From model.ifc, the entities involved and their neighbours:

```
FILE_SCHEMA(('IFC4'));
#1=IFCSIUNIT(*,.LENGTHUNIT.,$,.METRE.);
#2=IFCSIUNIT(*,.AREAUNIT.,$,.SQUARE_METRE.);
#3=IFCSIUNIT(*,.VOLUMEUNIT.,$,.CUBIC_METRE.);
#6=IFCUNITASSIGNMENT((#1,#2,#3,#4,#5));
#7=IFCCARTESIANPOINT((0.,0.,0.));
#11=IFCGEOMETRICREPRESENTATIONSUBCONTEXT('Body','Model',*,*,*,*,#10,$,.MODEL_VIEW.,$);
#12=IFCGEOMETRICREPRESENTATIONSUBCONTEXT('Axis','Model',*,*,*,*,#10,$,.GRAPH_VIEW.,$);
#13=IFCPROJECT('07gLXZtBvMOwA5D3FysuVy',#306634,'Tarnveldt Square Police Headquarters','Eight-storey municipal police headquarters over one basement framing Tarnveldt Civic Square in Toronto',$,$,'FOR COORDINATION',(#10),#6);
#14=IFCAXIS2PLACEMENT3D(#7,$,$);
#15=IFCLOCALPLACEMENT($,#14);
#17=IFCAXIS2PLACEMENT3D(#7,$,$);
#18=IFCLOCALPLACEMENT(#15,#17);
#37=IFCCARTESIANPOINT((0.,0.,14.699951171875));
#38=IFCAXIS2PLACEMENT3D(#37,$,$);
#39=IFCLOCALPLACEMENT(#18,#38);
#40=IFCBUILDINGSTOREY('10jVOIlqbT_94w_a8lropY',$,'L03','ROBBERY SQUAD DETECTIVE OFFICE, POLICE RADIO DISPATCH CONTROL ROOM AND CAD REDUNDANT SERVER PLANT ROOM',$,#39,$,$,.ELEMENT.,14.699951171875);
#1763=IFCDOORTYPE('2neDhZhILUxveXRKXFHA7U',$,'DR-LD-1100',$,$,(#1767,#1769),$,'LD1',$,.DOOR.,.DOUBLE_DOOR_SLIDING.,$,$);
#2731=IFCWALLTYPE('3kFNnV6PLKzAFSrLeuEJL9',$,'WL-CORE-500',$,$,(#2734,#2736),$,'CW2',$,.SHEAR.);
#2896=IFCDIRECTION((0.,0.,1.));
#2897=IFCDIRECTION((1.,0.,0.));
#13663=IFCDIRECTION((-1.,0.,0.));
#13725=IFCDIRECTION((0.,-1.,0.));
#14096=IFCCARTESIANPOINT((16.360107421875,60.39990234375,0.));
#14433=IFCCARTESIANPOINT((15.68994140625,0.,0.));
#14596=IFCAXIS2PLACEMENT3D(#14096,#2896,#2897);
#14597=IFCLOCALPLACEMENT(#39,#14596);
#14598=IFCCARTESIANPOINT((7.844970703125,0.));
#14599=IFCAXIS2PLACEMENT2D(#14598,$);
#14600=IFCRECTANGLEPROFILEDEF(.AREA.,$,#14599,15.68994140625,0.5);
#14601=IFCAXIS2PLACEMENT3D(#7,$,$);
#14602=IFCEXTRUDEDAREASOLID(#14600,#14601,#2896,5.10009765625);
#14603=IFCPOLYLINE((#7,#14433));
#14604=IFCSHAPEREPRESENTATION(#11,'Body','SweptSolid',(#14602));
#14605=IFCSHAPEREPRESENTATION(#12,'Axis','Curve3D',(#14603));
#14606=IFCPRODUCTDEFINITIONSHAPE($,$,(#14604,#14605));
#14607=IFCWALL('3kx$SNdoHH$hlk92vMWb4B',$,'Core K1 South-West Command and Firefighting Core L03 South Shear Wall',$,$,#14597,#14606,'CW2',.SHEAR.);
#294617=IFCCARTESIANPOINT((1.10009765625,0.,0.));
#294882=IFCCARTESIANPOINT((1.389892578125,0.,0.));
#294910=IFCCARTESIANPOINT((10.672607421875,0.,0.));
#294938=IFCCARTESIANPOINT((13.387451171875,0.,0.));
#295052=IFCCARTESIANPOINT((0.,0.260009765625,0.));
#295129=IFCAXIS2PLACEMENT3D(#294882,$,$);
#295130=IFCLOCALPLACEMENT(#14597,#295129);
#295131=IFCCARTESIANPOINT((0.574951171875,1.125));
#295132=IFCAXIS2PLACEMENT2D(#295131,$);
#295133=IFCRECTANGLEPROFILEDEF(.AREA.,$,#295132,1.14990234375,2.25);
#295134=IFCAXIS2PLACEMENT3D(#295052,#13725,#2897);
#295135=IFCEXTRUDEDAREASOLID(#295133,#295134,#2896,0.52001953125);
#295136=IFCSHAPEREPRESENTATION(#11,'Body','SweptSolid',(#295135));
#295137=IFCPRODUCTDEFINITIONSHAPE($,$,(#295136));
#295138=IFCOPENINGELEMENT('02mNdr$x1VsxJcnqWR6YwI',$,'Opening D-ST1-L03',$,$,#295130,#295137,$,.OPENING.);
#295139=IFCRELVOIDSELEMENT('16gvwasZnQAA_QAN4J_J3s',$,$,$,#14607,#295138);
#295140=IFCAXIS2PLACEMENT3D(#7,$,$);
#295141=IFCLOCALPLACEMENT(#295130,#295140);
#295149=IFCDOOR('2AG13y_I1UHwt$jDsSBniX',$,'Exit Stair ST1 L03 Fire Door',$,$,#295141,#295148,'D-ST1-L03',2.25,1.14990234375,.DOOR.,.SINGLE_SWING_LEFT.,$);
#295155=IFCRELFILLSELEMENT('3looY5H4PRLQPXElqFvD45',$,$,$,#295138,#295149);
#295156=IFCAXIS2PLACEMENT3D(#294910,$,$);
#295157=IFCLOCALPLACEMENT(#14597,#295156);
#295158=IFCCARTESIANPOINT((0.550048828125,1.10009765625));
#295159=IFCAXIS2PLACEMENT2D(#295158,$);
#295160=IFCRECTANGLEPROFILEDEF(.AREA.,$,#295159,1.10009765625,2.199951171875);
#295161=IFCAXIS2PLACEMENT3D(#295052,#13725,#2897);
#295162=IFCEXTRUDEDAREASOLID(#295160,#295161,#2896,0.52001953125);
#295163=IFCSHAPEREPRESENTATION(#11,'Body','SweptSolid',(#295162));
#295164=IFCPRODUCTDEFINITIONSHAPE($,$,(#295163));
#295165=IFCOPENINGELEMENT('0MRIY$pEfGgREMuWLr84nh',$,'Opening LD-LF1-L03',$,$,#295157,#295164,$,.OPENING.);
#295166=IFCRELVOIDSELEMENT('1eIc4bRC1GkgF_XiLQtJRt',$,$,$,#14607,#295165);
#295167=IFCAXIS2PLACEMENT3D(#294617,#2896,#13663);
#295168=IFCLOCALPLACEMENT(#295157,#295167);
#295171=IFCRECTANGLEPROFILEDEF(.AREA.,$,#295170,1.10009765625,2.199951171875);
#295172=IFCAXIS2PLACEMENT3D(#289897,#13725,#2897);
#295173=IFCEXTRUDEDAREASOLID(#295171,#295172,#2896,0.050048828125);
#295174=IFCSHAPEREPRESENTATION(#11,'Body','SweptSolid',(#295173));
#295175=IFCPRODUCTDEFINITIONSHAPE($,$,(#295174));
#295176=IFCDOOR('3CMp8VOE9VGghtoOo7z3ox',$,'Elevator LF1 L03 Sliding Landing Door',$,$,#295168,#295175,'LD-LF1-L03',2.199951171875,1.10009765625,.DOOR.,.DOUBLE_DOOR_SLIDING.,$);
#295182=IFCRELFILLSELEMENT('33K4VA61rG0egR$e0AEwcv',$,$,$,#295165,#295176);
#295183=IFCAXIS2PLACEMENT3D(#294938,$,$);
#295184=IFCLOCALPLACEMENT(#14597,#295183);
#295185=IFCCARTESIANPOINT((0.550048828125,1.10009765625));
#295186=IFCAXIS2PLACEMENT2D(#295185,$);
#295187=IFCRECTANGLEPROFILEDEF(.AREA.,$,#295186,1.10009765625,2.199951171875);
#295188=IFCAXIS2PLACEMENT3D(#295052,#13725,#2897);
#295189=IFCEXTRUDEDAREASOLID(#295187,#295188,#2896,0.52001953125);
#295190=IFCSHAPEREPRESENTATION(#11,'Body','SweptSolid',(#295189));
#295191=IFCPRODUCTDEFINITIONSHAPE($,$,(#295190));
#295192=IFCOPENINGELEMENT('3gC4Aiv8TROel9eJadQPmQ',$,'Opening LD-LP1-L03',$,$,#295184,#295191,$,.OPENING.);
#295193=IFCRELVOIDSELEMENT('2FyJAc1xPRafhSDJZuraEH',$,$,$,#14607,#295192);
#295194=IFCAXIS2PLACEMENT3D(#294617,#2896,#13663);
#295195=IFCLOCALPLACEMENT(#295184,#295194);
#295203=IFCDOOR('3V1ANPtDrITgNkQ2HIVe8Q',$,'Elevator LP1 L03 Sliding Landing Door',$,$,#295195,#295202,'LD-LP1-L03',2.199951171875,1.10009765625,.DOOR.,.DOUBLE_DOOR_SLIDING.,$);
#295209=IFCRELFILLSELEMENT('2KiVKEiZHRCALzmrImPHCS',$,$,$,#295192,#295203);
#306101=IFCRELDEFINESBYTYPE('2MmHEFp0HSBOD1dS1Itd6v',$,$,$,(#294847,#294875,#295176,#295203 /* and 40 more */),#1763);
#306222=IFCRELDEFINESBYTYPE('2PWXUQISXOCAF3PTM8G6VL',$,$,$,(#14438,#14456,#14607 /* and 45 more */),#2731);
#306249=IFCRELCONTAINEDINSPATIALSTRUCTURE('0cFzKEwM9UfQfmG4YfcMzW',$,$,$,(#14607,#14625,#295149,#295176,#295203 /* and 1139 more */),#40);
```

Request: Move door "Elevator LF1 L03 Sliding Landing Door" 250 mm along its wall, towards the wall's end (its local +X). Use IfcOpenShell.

```python
import ifcopenshell
import ifcopenshell.api.geometry
import ifcopenshell.util.placement
import ifcopenshell.util.unit

model = ifcopenshell.open("model.ifc")
unit_scale = ifcopenshell.util.unit.calculate_unit_scale(model)

door = model.by_guid("3CMp8VOE9VGghtoOo7z3ox")
opening = door.FillsVoids[0].RelatingOpeningElement
wall = opening.VoidsElements[0].RelatingBuildingElement

wall_matrix = ifcopenshell.util.placement.get_local_placement(wall.ObjectPlacement)
shift = wall_matrix[:3, 0] * 0.25 / unit_scale
before = ifcopenshell.util.placement.get_local_placement(door.ObjectPlacement)[:3, 3].copy()

# The door is placed relative to its opening, so it follows when the opening moves.
matrix = ifcopenshell.util.placement.get_local_placement(opening.ObjectPlacement)
matrix[:3, 3] += shift
ifcopenshell.api.geometry.edit_object_placement(
    model, product=opening, matrix=matrix, is_si=False, should_transform_children=True
)

after = ifcopenshell.util.placement.get_local_placement(door.ObjectPlacement)[:3, 3]
print("door moved by", (after - before).round(3) + 0.0)

model.write("model_edited.ifc")
```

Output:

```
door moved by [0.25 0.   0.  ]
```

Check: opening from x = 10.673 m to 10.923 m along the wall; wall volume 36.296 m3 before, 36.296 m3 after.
